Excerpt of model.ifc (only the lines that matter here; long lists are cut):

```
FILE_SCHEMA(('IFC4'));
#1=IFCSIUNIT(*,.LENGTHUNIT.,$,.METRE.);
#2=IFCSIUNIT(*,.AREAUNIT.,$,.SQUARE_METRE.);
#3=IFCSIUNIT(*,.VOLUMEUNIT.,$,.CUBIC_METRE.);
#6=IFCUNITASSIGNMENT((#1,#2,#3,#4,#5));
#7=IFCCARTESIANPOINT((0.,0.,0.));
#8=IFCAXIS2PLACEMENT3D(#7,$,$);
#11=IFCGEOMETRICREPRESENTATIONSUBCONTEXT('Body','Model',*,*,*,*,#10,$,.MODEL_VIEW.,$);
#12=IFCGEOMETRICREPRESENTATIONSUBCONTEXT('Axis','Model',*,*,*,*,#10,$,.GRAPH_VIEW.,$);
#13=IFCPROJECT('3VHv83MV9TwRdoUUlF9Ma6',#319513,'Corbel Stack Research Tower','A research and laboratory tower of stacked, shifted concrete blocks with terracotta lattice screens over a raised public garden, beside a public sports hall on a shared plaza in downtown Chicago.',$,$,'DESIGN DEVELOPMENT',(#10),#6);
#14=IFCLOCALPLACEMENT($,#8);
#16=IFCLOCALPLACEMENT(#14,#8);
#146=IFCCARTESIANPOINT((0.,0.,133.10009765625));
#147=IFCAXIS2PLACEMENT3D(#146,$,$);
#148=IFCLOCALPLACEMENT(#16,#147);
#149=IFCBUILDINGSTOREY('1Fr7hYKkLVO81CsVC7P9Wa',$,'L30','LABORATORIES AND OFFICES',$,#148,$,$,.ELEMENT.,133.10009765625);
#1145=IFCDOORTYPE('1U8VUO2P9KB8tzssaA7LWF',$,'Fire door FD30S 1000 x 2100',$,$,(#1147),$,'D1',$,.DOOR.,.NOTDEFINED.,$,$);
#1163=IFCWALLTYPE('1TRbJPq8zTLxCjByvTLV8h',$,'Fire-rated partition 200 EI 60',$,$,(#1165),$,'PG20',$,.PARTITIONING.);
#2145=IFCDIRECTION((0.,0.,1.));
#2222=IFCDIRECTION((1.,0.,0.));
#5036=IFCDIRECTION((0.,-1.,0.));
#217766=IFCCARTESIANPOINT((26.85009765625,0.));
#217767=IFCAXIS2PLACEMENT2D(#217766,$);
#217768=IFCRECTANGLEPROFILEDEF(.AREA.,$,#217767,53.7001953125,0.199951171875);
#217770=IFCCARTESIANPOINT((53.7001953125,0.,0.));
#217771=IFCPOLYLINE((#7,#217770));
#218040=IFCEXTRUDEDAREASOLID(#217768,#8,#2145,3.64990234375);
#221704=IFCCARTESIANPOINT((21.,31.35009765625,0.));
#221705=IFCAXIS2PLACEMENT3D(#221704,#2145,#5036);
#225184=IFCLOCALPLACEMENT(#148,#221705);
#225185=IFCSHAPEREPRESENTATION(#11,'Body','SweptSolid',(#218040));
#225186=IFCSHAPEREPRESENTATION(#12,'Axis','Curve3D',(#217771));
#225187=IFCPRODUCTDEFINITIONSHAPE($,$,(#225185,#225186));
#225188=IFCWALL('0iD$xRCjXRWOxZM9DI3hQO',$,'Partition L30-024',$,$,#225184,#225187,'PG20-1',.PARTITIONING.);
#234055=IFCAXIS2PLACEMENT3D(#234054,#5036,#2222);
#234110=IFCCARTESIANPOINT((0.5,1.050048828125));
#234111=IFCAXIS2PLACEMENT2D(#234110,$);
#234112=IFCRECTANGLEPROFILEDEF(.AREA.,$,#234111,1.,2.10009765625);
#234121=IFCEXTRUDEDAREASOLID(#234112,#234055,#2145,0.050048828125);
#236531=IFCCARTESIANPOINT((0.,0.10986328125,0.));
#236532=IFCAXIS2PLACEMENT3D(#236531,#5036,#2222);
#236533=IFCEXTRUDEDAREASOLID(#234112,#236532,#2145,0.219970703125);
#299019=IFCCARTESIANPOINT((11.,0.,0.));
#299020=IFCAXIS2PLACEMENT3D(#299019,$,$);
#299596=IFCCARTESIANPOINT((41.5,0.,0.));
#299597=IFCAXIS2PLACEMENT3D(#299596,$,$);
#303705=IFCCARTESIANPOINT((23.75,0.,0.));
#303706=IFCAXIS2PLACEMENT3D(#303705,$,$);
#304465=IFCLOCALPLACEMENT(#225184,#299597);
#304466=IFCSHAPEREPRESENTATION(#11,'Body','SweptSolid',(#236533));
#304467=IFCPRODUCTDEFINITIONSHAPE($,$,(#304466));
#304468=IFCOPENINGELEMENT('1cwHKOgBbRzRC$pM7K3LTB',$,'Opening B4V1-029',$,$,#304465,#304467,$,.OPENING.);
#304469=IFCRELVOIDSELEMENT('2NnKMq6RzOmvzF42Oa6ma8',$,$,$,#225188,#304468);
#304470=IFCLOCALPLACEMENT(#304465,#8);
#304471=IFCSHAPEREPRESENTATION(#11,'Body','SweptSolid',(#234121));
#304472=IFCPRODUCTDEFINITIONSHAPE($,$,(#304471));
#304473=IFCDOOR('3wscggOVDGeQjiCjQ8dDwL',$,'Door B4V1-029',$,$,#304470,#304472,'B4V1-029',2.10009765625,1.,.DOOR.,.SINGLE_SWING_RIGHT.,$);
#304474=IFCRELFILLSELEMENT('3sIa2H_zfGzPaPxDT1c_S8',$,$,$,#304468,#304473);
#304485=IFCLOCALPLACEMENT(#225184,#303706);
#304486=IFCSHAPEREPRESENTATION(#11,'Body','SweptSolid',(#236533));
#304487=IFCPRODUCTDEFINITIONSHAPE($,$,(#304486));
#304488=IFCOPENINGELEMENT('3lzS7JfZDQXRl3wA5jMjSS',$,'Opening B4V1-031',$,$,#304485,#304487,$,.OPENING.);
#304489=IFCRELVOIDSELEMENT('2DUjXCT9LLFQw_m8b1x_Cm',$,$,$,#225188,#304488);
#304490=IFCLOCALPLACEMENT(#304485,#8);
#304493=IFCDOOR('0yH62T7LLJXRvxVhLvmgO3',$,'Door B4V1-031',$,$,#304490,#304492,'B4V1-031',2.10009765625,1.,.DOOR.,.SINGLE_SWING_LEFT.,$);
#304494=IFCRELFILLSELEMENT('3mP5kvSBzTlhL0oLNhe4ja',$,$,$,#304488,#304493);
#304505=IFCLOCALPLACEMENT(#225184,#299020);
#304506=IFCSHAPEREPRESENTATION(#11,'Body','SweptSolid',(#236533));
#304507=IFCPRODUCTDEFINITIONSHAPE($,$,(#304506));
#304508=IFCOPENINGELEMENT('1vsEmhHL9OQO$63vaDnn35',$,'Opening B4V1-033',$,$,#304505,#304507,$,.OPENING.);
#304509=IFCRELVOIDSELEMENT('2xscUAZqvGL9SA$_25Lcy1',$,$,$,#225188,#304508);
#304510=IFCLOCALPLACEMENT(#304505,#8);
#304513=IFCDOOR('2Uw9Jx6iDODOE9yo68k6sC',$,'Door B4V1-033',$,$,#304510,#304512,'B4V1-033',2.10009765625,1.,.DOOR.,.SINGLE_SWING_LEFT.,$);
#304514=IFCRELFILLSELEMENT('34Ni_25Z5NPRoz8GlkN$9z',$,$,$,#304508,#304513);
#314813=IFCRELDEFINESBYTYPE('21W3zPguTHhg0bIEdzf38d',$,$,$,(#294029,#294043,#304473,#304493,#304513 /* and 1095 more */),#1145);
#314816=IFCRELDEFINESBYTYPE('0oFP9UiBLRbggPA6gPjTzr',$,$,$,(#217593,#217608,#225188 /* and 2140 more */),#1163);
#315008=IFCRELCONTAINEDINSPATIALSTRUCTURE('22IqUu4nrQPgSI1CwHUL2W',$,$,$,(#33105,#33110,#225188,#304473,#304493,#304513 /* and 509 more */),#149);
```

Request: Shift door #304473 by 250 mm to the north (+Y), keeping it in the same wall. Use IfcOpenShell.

```python
import ifcopenshell
import ifcopenshell.api.geometry
import ifcopenshell.util.placement
import ifcopenshell.util.unit

model = ifcopenshell.open("model.ifc")
unit_scale = ifcopenshell.util.unit.calculate_unit_scale(model)

door = model.by_id(304473)
opening = door.FillsVoids[0].RelatingOpeningElement
wall = opening.VoidsElements[0].RelatingBuildingElement

wall_matrix = ifcopenshell.util.placement.get_local_placement(wall.ObjectPlacement)
shift = wall_matrix[:3, 0] * -0.25 / unit_scale
before = ifcopenshell.util.placement.get_local_placement(door.ObjectPlacement)[:3, 3].copy()

# The door is placed relative to its opening, so it follows when the opening moves.
matrix = ifcopenshell.util.placement.get_local_placement(opening.ObjectPlacement)
matrix[:3, 3] += shift
ifcopenshell.api.geometry.edit_object_placement(
    model, product=opening, matrix=matrix, is_si=False, should_transform_children=True
)

after = ifcopenshell.util.placement.get_local_placement(door.ObjectPlacement)[:3, 3]
print("door moved by", (after - before).round(3) + 0.0)

model.write("model_rev.ifc")
```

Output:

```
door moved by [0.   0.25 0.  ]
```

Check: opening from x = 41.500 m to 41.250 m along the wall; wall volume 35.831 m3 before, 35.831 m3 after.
